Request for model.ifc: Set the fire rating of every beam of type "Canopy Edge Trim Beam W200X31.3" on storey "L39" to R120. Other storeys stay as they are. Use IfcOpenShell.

First a look at what the model holds.

```python
import ifcopenshell
import ifcopenshell.util.element

model = ifcopenshell.open("model.ifc")
print(model.schema)
storey = next(s for s in model.by_type("IfcBuildingStorey") if s.Name == "L39")
beams = [e for e in ifcopenshell.util.element.get_decomposition(storey) if e.is_a("IfcBeam")]
seen = {}
for e in beams:
    element_type = ifcopenshell.util.element.get_type(e)
    key = (element_type.Name if element_type != e and element_type else None, ifcopenshell.util.element.get_pset(e, "Pset_BeamCommon", "FireRating"))
    seen[key] = seen.get(key, 0) + 1
for (name, value), count in sorted(seen.items(), key=str):
    print(count, "x", name, "|", value)
```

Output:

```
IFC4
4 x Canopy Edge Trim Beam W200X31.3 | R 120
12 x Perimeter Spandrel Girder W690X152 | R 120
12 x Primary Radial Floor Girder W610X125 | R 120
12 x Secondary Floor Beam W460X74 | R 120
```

```python
import ifcopenshell
import ifcopenshell.api.pset
import ifcopenshell.util.element

model = ifcopenshell.open("model.ifc")

storey = next(s for s in model.by_type("IfcBuildingStorey") if s.Name == "L39")
beams = [e for e in ifcopenshell.util.element.get_decomposition(storey) if e.is_a("IfcBeam")]

count = 0
for e in beams:
    element_type = ifcopenshell.util.element.get_type(e)
    if element_type in (None, e) or element_type.Name != "Canopy Edge Trim Beam W200X31.3":
        continue
    # add_pset returns the element's existing set when there is one.
    pset = ifcopenshell.api.pset.add_pset(model, product=e, name="Pset_BeamCommon")
    ifcopenshell.api.pset.edit_pset(model, pset=pset, properties={"FireRating": "R120"})
    count += 1

print(count, "beams updated")

model.write("model_updated.ifc")
```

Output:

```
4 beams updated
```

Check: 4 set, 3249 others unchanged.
